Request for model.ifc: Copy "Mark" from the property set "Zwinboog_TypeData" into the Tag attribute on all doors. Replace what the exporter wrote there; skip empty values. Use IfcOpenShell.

First a look at what the model holds.

```python
import ifcopenshell
import ifcopenshell.util.element

model = ifcopenshell.open("model.ifc")
print(model.schema)
doors = model.by_type("IfcDoor")
print(len(doors), "doors")
for e in doors[:8]:
    source = ifcopenshell.util.element.get_pset(e, "Zwinboog_TypeData", "Mark")
    target = e.Tag
    print(e.id(), repr(source), repr(target), sep=" | ")
```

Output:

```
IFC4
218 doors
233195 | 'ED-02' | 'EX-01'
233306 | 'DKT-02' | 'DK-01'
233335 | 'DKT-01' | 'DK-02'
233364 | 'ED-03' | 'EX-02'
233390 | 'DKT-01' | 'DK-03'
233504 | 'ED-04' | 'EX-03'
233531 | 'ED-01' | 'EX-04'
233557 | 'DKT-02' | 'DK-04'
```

```python
import ifcopenshell
import ifcopenshell.util.element

model = ifcopenshell.open("model.ifc")

count = 0
for e in model.by_type("IfcDoor"):
    value = ifcopenshell.util.element.get_pset(e, "Zwinboog_TypeData", "Mark")
    current = e.Tag
    if not value or not value.strip() or current == value:
        continue
    e.Tag = value
    count += 1

print(count, "doors updated")

model.write("model-out.ifc")
```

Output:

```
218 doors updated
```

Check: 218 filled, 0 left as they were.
